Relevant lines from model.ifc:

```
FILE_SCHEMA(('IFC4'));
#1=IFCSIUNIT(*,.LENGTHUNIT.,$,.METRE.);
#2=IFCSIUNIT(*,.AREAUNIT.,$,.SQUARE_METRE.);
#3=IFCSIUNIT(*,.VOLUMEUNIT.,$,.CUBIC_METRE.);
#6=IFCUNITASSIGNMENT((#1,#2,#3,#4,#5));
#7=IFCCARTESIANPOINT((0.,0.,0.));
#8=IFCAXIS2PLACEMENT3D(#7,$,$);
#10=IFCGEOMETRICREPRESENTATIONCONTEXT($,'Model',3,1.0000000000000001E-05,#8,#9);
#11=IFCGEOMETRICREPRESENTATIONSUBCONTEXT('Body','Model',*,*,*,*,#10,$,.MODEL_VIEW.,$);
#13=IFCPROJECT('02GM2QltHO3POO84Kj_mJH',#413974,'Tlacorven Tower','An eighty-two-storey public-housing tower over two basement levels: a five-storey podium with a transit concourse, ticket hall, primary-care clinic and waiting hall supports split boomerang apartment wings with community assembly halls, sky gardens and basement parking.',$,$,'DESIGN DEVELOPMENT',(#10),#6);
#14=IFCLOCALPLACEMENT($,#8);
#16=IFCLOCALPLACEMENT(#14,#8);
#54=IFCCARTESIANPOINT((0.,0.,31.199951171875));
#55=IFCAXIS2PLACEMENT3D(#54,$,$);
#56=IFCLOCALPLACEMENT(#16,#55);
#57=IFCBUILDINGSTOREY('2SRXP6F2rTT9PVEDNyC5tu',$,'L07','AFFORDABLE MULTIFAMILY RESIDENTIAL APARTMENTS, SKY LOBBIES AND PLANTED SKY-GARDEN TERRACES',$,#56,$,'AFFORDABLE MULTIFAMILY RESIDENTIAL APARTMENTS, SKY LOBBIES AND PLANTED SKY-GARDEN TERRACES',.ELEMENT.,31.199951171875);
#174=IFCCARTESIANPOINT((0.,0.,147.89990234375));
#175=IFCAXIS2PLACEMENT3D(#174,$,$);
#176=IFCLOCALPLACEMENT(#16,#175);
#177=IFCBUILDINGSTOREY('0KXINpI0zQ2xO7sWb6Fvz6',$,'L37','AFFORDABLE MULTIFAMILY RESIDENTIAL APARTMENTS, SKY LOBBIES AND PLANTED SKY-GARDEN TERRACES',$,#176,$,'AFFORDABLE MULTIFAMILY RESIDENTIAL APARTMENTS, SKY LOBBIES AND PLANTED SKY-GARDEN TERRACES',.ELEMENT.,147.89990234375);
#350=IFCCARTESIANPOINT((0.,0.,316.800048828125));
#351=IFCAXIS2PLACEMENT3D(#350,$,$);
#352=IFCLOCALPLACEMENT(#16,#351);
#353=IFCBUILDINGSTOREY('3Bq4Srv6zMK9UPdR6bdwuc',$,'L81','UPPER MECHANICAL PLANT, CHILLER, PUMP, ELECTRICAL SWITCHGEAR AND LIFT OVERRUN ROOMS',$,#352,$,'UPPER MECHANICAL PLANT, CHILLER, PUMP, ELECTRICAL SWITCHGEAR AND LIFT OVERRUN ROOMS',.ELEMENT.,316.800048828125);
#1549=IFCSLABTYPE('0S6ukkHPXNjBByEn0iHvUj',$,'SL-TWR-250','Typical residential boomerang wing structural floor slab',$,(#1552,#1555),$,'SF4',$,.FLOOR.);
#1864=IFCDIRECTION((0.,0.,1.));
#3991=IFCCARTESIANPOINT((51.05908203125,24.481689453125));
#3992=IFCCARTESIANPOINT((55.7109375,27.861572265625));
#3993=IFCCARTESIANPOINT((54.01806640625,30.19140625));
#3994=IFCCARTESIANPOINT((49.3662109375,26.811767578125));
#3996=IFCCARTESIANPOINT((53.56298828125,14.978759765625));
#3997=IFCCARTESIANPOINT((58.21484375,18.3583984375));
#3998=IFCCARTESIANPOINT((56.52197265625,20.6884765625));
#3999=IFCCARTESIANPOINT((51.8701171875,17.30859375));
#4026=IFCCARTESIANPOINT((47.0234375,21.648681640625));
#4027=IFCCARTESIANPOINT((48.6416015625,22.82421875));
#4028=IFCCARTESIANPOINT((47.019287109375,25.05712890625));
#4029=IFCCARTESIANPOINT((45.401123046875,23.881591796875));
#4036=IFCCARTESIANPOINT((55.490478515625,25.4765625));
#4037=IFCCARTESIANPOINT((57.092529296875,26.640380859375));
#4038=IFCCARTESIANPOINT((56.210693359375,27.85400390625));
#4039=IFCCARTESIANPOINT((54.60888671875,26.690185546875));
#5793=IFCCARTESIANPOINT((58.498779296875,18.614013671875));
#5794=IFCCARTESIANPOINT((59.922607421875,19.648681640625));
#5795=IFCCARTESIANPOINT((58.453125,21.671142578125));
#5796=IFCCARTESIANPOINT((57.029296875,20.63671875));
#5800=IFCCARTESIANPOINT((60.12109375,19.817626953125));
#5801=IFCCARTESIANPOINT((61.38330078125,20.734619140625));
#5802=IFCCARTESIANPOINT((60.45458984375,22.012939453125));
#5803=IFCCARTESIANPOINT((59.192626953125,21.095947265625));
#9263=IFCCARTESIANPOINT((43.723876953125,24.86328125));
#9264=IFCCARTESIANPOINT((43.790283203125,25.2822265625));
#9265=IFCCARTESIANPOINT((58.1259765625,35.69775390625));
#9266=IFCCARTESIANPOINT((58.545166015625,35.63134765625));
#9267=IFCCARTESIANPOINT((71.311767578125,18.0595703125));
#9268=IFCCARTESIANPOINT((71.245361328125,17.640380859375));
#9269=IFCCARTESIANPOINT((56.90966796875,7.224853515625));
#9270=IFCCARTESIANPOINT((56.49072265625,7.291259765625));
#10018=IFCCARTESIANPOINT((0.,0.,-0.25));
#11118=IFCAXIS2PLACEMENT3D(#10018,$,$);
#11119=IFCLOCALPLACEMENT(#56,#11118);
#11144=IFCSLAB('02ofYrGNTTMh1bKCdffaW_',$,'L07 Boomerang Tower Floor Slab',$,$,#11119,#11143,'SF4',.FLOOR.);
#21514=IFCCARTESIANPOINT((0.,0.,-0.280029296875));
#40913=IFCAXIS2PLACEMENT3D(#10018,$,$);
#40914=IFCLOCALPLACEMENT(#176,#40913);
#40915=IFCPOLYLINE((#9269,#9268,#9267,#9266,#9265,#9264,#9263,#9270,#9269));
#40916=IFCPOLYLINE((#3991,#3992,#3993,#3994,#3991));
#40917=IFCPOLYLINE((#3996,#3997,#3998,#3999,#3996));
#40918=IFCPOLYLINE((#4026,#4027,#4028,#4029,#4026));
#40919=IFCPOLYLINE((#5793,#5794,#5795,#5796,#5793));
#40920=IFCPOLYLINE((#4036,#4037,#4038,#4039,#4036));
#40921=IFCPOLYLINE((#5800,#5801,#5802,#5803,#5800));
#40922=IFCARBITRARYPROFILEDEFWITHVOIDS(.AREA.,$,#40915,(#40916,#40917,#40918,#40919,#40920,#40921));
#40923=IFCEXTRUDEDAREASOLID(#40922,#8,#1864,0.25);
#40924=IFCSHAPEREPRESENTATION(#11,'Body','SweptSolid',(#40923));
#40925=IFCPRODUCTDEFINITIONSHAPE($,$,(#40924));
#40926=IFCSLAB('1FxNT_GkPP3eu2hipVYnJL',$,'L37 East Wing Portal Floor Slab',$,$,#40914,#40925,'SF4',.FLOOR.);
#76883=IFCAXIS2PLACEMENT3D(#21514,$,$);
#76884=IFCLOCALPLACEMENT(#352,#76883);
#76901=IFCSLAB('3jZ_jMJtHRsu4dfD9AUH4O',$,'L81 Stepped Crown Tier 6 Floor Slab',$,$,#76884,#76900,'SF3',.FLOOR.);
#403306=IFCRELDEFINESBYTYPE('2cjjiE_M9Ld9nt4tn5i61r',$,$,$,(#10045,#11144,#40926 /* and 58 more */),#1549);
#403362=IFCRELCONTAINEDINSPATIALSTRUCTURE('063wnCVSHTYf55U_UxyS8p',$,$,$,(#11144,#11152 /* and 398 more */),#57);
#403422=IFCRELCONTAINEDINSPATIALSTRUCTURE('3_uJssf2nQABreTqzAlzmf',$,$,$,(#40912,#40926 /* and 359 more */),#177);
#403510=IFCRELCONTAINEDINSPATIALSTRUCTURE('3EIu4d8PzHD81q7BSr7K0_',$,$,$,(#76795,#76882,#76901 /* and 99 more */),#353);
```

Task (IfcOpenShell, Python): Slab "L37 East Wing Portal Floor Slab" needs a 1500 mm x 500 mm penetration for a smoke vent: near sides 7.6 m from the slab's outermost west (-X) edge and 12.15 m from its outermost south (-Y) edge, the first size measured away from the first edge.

```python
import numpy as np
import ifcopenshell
import ifcopenshell.api.feature
import ifcopenshell.api.geometry
import ifcopenshell.api.root
import ifcopenshell.geom
import ifcopenshell.util.placement
import ifcopenshell.util.representation
import ifcopenshell.util.shape
import ifcopenshell.util.unit

model = ifcopenshell.open("model.ifc")
unit_scale = ifcopenshell.util.unit.calculate_unit_scale(model)
settings = ifcopenshell.geom.settings()


def volume(element):
    """Net volume in cubic metres, openings subtracted."""
    shape = ifcopenshell.geom.create_shape(settings, element)
    return ifcopenshell.util.shape.get_volume(shape.geometry)


slab = model.by_guid("1FxNT_GkPP3eu2hipVYnJL")
before = volume(slab)

# Extent in the slab's own axes, in metres. The edges named are its -X and -Y sides.
slab_shape = ifcopenshell.geom.create_shape(settings, slab)
vertices = ifcopenshell.util.shape.get_vertices(slab_shape.geometry)
x_min, y_min, bottom = vertices.min(axis=0)
top = vertices[:, 2].max()

opening = ifcopenshell.api.root.create_entity(model, ifc_class="IfcOpeningElement", name="Smoke vent opening", predefined_type="OPENING")
context = ifcopenshell.util.representation.get_context(model, "Model", "Body", "MODEL_VIEW")
width, depth = 1.5, 0.5
outline = [(0.0, 0.0), (width, 0.0), (width, depth), (0.0, depth), (0.0, 0.0)]
# Overshoot both faces by 50 mm so the cut is clean.
shape = ifcopenshell.api.geometry.add_slab_representation(
    model, context=context, depth=top - bottom + 0.1, polyline=outline
)
ifcopenshell.api.geometry.assign_representation(model, product=opening, representation=shape)

matrix = ifcopenshell.util.placement.get_local_placement(slab.ObjectPlacement)
matrix[:, 3] = matrix @ np.append(np.array([x_min + 7.6, y_min + 12.15, bottom - 0.05]) / unit_scale, 1.0)
ifcopenshell.api.geometry.edit_object_placement(model, product=opening, matrix=matrix, is_si=False)
ifcopenshell.api.feature.add_feature(model, feature=opening, element=slab)

after = volume(slab)

print(f"slab volume {before:.3f} -> {after:.3f} m3")

model.write("model_updated.ifc")
```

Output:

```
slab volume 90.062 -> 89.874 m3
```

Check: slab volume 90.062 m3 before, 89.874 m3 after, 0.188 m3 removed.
